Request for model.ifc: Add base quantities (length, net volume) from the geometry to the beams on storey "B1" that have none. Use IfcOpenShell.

First a look at what the model holds.

```python
import ifcopenshell
import ifcopenshell.util.element
import ifcopenshell.util.unit

model = ifcopenshell.open("model.ifc")
print(model.schema)
for unit_type in ("LENGTHUNIT", "AREAUNIT", "VOLUMEUNIT"):
    print(unit_type, ifcopenshell.util.unit.calculate_unit_scale(model, unit_type))
storey = next(s for s in model.by_type("IfcBuildingStorey") if s.Name == "B1")
beams = [e for e in ifcopenshell.util.element.get_decomposition(storey) if e.is_a("IfcBeam")]
for e in sorted(beams, key=lambda e: e.id()):
    print(e.id(), e.is_a(), e.Name, list(ifcopenshell.util.element.get_psets(e, qtos_only=True)), sep=" | ")
```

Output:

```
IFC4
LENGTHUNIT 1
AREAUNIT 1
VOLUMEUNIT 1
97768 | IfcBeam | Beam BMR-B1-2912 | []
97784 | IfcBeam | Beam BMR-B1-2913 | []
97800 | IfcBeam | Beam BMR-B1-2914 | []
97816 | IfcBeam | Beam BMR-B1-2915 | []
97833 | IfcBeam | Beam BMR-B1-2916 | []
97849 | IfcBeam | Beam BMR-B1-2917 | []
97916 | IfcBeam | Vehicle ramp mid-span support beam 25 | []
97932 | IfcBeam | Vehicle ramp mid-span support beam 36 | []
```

```python
import ifcopenshell
import ifcopenshell.api.pset
import ifcopenshell.geom
import ifcopenshell.util.element
import ifcopenshell.util.shape
import ifcopenshell.util.unit

model = ifcopenshell.open("model.ifc")
unit_scale = ifcopenshell.util.unit.calculate_unit_scale(model)
volume_scale = ifcopenshell.util.unit.calculate_unit_scale(model, "VOLUMEUNIT")
settings = ifcopenshell.geom.settings()

storey = next(s for s in model.by_type("IfcBuildingStorey") if s.Name == "B1")
beams = [e for e in ifcopenshell.util.element.get_decomposition(storey) if e.is_a("IfcBeam")]

for e in sorted(beams, key=lambda e: e.id()):
    if ifcopenshell.util.element.get_psets(e, qtos_only=True, should_inherit=False):
        continue
    # Geometry comes back in metres, in the element's own axes.
    shape = ifcopenshell.geom.create_shape(settings, e)
    values = {
        "Length": ifcopenshell.util.shape.get_max_xyz(shape.geometry) / unit_scale,
        "NetVolume": ifcopenshell.util.shape.get_volume(shape.geometry) / volume_scale,
    }
    qto = ifcopenshell.api.pset.add_qto(model, product=e, name="Qto_BeamBaseQuantities")
    ifcopenshell.api.pset.edit_qto(model, qto=qto, properties=values)
    print(e.id(), {k: round(v, 3) for k, v in values.items()})

model.write("model_v2.ifc")
```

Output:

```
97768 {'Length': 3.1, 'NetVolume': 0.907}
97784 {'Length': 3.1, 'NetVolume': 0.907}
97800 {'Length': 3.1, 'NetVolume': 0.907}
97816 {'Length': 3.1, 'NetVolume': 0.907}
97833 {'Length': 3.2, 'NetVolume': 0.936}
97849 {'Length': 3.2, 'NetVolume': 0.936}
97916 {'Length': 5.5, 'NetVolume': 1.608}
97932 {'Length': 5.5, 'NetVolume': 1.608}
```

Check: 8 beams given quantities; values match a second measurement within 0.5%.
